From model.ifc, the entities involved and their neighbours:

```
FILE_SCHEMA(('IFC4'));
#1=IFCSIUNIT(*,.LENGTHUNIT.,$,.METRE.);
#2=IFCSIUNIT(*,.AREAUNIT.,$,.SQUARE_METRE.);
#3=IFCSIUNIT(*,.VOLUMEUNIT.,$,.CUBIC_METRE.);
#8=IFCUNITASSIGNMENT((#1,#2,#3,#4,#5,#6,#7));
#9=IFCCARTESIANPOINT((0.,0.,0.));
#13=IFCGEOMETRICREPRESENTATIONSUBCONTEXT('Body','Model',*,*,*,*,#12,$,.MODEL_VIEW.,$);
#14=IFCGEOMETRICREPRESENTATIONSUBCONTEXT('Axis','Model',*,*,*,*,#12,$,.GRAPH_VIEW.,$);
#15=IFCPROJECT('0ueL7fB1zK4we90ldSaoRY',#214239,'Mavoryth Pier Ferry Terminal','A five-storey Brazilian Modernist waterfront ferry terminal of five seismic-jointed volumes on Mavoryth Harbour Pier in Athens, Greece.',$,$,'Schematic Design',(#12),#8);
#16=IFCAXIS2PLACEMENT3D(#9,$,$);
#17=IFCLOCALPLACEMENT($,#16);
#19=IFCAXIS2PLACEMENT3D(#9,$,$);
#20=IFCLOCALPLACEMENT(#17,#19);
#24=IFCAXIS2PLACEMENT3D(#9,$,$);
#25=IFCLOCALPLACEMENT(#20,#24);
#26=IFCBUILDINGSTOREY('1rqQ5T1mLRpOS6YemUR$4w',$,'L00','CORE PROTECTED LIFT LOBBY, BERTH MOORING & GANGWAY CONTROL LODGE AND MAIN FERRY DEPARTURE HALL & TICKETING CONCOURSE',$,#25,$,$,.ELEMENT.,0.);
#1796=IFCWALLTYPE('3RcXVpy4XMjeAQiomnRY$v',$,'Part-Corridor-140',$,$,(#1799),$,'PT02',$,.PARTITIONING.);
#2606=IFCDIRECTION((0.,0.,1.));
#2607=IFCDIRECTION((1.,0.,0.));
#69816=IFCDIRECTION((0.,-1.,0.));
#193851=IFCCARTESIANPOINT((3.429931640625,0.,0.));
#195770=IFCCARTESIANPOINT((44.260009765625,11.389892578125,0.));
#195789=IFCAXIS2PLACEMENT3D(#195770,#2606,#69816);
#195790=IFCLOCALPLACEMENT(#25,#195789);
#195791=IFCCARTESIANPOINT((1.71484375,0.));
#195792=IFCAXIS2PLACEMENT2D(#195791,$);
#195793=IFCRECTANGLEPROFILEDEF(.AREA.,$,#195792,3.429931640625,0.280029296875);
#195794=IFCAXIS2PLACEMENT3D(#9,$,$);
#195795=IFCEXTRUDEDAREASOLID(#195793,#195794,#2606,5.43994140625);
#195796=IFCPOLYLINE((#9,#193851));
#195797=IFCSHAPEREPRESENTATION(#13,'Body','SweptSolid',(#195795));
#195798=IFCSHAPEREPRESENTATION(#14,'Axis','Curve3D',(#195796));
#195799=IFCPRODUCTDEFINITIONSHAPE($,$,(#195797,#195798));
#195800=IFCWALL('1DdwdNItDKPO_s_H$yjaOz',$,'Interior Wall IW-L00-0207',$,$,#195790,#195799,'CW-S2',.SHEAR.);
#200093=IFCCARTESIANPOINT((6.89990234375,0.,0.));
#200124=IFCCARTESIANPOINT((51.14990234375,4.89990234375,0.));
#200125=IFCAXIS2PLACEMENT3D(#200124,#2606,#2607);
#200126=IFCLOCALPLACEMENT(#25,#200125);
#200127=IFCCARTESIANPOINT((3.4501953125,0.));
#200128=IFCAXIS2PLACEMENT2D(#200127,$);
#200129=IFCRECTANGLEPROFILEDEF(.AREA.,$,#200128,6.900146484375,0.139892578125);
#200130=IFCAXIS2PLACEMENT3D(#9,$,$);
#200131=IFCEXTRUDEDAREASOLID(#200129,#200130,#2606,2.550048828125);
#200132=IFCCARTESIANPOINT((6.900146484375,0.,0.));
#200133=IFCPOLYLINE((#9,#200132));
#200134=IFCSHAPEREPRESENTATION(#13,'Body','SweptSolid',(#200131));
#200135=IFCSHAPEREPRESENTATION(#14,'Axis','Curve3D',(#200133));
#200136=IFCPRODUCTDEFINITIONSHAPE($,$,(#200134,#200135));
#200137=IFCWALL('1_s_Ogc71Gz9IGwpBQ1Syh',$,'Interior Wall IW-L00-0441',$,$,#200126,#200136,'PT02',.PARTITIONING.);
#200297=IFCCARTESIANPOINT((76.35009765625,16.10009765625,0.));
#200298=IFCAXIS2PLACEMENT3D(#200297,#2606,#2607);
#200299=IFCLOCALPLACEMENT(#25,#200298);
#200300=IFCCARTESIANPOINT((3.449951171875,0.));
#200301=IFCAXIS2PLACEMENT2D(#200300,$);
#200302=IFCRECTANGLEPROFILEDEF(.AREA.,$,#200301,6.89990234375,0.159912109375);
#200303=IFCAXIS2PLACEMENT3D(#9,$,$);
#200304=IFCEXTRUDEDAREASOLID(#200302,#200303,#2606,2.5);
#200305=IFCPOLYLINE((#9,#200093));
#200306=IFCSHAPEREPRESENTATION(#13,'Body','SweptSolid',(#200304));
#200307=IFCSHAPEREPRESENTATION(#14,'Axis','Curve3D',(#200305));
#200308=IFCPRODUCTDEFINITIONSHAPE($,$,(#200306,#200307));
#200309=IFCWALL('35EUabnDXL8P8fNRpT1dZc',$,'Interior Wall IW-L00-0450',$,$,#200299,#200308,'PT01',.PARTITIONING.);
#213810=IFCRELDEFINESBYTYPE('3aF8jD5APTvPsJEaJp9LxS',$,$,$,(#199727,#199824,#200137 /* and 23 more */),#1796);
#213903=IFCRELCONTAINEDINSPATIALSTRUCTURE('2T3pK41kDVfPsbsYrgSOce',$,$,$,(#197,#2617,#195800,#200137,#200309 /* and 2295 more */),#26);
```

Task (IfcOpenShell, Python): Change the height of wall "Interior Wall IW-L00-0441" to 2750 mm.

```python
import ifcopenshell
import ifcopenshell.geom
import ifcopenshell.util.representation
import ifcopenshell.util.shape
import ifcopenshell.util.unit

model = ifcopenshell.open("model.ifc")
unit_scale = ifcopenshell.util.unit.calculate_unit_scale(model)
settings = ifcopenshell.geom.settings()


def volume(element):
    """Net volume in cubic metres, openings subtracted."""
    shape = ifcopenshell.geom.create_shape(settings, element)
    return ifcopenshell.util.shape.get_volume(shape.geometry)


wall = model.by_guid("1_s_Ogc71Gz9IGwpBQ1Syh")
before = volume(wall)

body = ifcopenshell.util.representation.get_representation(wall, "Model", "Body")
solid = body.Items[0]
old_height = solid.Depth
solid.Depth = 2.75 / unit_scale
after = volume(wall)

print(f"height {old_height:g} -> {solid.Depth:g}, volume {before:.3f} -> {after:.3f} m3")

model.write("model_edited.ifc")
```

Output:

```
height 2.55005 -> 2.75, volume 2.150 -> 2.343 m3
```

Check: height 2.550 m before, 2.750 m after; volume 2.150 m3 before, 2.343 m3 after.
